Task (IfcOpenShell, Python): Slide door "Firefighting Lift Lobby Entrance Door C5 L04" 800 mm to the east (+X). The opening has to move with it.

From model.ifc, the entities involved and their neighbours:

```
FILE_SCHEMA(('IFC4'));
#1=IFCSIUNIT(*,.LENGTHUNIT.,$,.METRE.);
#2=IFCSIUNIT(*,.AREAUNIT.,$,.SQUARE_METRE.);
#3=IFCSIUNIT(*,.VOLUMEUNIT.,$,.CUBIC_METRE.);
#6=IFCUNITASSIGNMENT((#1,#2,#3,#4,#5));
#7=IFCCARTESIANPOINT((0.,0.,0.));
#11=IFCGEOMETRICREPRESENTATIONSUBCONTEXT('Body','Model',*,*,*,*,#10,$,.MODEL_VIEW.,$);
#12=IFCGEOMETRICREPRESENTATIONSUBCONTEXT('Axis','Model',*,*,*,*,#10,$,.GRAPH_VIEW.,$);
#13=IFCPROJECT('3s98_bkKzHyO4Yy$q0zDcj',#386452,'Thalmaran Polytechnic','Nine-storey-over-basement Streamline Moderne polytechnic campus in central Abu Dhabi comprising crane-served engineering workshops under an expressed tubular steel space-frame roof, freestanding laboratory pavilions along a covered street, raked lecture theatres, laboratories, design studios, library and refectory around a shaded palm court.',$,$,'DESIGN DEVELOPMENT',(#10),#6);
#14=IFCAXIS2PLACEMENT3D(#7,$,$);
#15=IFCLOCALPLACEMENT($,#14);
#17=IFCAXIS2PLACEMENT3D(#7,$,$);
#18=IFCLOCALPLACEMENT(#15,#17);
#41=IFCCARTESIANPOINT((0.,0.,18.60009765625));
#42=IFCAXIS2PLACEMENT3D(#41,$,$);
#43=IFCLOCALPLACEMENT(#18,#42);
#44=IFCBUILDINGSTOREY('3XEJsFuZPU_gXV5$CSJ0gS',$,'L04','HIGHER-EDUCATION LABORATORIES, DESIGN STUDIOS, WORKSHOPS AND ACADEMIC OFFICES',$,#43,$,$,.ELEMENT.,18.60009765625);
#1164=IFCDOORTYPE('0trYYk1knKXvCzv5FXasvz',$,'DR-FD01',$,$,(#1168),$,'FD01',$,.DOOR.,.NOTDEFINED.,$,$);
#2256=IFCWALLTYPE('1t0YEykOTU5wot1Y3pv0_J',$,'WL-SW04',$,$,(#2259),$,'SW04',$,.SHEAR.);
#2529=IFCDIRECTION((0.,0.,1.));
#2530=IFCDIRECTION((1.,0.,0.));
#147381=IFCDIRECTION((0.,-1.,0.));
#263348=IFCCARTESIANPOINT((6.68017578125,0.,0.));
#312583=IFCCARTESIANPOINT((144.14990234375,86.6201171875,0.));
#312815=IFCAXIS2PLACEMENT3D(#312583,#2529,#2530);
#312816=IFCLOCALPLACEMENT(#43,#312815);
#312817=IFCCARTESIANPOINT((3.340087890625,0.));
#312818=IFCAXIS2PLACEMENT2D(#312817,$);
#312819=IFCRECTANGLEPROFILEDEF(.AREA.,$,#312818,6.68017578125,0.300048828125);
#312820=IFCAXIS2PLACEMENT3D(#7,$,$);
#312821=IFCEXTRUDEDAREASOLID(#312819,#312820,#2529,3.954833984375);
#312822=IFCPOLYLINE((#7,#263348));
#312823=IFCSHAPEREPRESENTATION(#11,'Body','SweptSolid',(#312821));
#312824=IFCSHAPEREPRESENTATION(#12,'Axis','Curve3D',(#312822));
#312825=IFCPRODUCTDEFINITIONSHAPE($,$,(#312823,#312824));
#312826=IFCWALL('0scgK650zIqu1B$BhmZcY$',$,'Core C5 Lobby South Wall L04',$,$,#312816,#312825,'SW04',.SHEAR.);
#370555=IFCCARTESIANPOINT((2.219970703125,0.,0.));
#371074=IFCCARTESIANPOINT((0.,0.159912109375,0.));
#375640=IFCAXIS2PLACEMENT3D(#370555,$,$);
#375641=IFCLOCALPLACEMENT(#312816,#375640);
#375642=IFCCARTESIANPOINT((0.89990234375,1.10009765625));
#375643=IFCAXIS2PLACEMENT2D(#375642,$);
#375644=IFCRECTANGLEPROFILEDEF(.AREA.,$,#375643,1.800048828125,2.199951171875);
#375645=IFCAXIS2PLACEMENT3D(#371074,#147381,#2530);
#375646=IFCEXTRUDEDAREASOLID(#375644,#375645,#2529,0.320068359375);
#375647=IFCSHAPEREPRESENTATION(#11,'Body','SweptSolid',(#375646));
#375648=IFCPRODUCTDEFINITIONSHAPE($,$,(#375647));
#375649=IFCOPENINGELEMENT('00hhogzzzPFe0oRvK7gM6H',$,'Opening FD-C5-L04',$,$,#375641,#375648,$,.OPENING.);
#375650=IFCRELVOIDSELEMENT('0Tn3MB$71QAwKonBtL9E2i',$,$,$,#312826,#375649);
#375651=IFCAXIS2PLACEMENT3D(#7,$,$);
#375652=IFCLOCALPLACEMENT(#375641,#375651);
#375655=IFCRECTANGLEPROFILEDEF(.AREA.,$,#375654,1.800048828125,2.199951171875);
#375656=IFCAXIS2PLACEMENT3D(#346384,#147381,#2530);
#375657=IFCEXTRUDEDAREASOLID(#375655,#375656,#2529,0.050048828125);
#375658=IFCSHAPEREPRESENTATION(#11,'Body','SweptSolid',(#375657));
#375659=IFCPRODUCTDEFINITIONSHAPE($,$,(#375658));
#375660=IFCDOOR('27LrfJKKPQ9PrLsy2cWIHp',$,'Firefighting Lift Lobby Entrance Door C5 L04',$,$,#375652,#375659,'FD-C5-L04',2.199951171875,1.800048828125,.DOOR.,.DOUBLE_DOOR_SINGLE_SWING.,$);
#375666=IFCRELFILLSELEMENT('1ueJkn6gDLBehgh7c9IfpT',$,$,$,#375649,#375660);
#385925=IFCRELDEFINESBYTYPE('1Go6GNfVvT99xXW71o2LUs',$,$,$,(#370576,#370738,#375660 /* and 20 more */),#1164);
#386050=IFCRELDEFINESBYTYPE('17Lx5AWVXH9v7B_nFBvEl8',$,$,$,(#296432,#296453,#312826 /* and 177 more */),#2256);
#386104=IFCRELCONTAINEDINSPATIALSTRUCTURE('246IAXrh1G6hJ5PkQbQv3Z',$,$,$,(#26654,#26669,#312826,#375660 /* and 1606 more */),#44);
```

```python
import ifcopenshell
import ifcopenshell.api.geometry
import ifcopenshell.util.placement
import ifcopenshell.util.unit

model = ifcopenshell.open("model.ifc")
unit_scale = ifcopenshell.util.unit.calculate_unit_scale(model)

door = model.by_id(375660)
opening = door.FillsVoids[0].RelatingOpeningElement
wall = opening.VoidsElements[0].RelatingBuildingElement

wall_matrix = ifcopenshell.util.placement.get_local_placement(wall.ObjectPlacement)
shift = wall_matrix[:3, 0] * 0.8 / unit_scale
before = ifcopenshell.util.placement.get_local_placement(door.ObjectPlacement)[:3, 3].copy()

# The door is placed relative to its opening, so it follows when the opening moves.
matrix = ifcopenshell.util.placement.get_local_placement(opening.ObjectPlacement)
matrix[:3, 3] += shift
ifcopenshell.api.geometry.edit_object_placement(
    model, product=opening, matrix=matrix, is_si=False, should_transform_children=True
)

after = ifcopenshell.util.placement.get_local_placement(door.ObjectPlacement)[:3, 3]
print("door moved by", (after - before).round(3) + 0.0)

model.write("model_edited.ifc")
```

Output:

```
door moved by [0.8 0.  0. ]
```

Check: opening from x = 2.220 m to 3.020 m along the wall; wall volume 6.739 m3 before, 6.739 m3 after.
